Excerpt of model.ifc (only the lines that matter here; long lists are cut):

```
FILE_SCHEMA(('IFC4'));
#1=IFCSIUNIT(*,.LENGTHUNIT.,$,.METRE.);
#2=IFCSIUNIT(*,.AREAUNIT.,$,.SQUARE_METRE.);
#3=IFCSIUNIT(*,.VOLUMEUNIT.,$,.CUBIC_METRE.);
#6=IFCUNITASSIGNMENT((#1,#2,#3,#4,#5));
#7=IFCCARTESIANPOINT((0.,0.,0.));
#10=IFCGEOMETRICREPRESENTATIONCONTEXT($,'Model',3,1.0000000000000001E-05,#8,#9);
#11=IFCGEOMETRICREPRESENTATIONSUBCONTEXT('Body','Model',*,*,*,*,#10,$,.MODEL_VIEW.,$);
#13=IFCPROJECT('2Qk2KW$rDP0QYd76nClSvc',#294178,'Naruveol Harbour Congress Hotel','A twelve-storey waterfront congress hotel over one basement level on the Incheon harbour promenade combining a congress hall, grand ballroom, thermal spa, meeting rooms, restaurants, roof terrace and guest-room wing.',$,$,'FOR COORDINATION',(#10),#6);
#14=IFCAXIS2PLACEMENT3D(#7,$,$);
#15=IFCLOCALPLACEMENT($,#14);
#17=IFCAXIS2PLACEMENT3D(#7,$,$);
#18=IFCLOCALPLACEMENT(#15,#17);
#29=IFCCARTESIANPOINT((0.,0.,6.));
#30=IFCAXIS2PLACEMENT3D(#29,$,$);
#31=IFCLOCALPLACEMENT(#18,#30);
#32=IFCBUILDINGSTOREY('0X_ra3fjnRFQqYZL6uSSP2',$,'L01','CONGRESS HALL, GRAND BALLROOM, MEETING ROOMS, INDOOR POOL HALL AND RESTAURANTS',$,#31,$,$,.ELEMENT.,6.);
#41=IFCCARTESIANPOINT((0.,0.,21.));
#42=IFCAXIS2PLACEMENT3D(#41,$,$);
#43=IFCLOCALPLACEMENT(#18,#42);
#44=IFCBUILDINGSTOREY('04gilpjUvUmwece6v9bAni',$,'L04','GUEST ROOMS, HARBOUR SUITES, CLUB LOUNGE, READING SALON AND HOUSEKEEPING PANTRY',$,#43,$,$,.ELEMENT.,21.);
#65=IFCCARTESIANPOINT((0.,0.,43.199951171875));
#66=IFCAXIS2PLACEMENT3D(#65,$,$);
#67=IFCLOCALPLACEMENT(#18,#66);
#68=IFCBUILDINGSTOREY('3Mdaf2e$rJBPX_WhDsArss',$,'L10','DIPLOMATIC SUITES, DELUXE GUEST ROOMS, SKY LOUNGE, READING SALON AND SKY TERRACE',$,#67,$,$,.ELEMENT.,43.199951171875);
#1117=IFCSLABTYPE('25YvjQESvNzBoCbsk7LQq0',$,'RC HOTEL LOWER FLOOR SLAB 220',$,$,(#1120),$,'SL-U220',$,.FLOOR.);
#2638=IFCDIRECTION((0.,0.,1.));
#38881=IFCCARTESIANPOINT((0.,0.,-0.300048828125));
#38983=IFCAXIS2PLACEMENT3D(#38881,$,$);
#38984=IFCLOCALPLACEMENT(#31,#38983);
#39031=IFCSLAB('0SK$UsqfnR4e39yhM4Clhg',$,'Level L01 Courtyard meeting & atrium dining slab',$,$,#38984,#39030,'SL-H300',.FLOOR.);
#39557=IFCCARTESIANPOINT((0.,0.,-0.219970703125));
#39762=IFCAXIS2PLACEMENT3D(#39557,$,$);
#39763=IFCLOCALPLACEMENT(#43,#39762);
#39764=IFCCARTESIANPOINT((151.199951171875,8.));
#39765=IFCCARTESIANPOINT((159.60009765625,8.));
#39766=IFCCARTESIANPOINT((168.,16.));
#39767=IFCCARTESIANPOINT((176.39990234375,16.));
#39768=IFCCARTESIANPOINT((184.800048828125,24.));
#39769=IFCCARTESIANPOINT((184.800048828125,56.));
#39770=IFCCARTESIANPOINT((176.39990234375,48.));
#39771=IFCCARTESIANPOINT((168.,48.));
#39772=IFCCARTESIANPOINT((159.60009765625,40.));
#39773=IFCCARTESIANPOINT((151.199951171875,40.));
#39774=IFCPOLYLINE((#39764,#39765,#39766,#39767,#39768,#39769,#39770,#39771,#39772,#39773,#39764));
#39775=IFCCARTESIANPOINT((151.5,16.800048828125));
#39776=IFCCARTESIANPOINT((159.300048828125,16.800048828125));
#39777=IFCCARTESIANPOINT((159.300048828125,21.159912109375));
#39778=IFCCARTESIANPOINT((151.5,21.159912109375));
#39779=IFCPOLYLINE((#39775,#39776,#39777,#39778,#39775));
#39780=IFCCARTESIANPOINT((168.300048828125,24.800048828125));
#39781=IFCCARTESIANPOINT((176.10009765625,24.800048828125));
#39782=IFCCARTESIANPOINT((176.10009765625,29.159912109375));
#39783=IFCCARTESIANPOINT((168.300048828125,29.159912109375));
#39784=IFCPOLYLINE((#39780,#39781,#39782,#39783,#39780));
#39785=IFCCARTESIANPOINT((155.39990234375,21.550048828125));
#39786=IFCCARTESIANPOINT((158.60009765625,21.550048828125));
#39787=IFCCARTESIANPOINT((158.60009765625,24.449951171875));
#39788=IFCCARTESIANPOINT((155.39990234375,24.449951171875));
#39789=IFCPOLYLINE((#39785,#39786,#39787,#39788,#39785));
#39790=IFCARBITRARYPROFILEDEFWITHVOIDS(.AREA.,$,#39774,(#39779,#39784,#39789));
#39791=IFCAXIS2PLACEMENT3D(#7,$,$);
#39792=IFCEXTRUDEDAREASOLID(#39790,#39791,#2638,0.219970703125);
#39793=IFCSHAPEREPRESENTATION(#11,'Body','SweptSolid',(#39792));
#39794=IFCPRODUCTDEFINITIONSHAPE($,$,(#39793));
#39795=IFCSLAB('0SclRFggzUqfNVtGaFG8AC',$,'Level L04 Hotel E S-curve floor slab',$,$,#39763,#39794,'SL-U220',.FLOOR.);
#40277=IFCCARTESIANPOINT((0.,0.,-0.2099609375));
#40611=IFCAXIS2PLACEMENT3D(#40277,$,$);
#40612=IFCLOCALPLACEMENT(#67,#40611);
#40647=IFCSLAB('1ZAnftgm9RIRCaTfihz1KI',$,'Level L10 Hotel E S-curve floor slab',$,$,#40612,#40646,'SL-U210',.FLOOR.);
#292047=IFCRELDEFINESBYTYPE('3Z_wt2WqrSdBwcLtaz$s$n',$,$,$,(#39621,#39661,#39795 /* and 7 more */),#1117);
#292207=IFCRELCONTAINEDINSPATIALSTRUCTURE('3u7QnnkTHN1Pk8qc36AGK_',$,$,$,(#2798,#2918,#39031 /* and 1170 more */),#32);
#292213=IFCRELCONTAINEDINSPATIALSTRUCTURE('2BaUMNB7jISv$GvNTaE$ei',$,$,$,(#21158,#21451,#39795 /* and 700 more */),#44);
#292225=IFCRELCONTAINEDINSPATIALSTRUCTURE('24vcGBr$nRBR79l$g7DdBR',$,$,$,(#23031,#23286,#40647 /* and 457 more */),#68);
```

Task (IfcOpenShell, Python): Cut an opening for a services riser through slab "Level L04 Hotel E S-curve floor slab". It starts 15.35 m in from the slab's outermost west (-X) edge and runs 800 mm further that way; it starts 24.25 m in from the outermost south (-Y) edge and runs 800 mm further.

```python
import numpy as np
import ifcopenshell
import ifcopenshell.api.feature
import ifcopenshell.api.geometry
import ifcopenshell.api.root
import ifcopenshell.geom
import ifcopenshell.util.placement
import ifcopenshell.util.representation
import ifcopenshell.util.shape
import ifcopenshell.util.unit

model = ifcopenshell.open("model.ifc")
unit_scale = ifcopenshell.util.unit.calculate_unit_scale(model)
settings = ifcopenshell.geom.settings()


def volume(element):
    """Net volume in cubic metres, openings subtracted."""
    shape = ifcopenshell.geom.create_shape(settings, element)
    return ifcopenshell.util.shape.get_volume(shape.geometry)


slab = model.by_guid("0SclRFggzUqfNVtGaFG8AC")
before = volume(slab)

# Extent in the slab's own axes, in metres. The edges named are its -X and -Y sides.
slab_shape = ifcopenshell.geom.create_shape(settings, slab)
vertices = ifcopenshell.util.shape.get_vertices(slab_shape.geometry)
x_min, y_min, bottom = vertices.min(axis=0)
top = vertices[:, 2].max()

opening = ifcopenshell.api.root.create_entity(model, ifc_class="IfcOpeningElement", name="Services riser opening", predefined_type="OPENING")
context = ifcopenshell.util.representation.get_context(model, "Model", "Body", "MODEL_VIEW")
width, depth = 0.8, 0.8
outline = [(0.0, 0.0), (width, 0.0), (width, depth), (0.0, depth), (0.0, 0.0)]
# Overshoot both faces by 50 mm so the cut is clean.
shape = ifcopenshell.api.geometry.add_slab_representation(
    model, context=context, depth=top - bottom + 0.1, polyline=outline
)
ifcopenshell.api.geometry.assign_representation(model, product=opening, representation=shape)

matrix = ifcopenshell.util.placement.get_local_placement(slab.ObjectPlacement)
matrix[:, 3] = matrix @ np.append(np.array([x_min + 15.35, y_min + 24.25, bottom - 0.05]) / unit_scale, 1.0)
ifcopenshell.api.geometry.edit_object_placement(model, product=opening, matrix=matrix, is_si=False)
ifcopenshell.api.feature.add_feature(model, feature=opening, element=slab)

after = volume(slab)

print(f"slab volume {before:.3f} -> {after:.3f} m3")

model.write("model-out.ifc")
```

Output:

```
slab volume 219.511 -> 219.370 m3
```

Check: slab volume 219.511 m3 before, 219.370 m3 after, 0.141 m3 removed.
